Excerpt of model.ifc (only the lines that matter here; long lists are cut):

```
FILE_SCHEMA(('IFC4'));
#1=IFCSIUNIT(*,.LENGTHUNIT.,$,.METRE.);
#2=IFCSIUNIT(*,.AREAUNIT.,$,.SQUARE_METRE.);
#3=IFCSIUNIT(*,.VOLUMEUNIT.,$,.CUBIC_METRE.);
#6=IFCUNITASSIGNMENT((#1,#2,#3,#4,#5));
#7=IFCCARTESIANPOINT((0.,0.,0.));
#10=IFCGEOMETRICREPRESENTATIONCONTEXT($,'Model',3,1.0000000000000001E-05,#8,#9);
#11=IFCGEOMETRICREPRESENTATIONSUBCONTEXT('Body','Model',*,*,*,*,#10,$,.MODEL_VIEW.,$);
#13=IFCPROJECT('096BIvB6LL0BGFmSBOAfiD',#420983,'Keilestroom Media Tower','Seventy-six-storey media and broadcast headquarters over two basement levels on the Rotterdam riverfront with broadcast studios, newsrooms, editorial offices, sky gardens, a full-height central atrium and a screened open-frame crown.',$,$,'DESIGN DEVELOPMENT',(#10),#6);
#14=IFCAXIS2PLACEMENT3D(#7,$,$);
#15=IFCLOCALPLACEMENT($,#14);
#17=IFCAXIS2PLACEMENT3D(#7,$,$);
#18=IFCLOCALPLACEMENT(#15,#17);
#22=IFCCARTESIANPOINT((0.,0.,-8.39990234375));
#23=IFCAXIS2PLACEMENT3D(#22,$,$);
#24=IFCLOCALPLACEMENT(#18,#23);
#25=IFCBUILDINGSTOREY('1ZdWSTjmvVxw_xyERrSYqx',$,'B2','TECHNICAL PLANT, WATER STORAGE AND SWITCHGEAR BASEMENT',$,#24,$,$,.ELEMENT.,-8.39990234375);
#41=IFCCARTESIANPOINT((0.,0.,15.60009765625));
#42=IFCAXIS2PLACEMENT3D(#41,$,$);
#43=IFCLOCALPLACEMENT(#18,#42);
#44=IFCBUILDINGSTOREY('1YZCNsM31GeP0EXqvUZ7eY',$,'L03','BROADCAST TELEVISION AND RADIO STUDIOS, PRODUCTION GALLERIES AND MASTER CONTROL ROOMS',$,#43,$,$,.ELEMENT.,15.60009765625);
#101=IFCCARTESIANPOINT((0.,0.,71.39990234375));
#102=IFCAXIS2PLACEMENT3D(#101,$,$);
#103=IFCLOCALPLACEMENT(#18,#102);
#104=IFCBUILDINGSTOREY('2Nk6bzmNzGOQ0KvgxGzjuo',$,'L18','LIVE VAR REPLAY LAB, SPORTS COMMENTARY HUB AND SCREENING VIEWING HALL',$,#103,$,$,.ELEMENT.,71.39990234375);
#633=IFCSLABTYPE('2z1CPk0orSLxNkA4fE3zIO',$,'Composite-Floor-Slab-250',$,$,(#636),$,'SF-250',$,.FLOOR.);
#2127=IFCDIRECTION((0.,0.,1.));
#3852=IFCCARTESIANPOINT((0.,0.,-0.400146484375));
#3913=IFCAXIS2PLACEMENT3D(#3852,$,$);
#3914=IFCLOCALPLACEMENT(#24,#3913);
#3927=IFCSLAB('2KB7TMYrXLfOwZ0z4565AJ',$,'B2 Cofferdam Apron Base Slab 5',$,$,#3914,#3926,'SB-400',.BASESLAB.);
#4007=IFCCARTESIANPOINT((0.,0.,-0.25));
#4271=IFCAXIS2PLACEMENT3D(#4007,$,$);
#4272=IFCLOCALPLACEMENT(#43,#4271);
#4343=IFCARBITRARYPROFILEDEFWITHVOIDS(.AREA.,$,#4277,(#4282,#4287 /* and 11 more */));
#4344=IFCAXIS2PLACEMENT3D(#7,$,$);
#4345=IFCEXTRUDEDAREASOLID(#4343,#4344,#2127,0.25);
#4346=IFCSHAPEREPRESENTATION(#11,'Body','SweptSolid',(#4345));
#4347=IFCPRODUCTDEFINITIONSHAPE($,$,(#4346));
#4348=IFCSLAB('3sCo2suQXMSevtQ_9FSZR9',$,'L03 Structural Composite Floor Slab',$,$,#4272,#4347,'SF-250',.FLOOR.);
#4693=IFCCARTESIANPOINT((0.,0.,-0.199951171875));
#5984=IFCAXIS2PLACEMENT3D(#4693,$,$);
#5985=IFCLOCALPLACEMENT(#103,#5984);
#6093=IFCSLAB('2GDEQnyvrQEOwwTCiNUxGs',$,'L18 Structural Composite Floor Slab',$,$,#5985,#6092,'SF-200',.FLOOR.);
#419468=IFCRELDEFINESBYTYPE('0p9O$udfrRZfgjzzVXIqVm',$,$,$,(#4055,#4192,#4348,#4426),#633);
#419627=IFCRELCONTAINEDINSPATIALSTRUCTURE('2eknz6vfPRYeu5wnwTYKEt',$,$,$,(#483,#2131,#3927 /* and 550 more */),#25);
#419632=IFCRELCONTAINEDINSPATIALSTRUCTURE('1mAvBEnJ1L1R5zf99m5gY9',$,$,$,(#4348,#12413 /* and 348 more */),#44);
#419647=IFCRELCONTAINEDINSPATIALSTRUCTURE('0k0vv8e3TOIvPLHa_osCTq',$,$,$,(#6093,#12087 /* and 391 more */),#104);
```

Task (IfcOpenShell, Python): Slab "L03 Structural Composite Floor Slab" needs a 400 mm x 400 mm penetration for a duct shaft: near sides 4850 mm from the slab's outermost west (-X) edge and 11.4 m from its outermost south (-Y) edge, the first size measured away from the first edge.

```python
import numpy as np
import ifcopenshell
import ifcopenshell.api.feature
import ifcopenshell.api.geometry
import ifcopenshell.api.root
import ifcopenshell.geom
import ifcopenshell.util.placement
import ifcopenshell.util.representation
import ifcopenshell.util.shape
import ifcopenshell.util.unit

model = ifcopenshell.open("model.ifc")
unit_scale = ifcopenshell.util.unit.calculate_unit_scale(model)
settings = ifcopenshell.geom.settings()


def volume(element):
    """Net volume in cubic metres, openings subtracted."""
    shape = ifcopenshell.geom.create_shape(settings, element)
    return ifcopenshell.util.shape.get_volume(shape.geometry)


slab = model.by_guid("3sCo2suQXMSevtQ_9FSZR9")
before = volume(slab)

# Extent in the slab's own axes, in metres. The edges named are its -X and -Y sides.
slab_shape = ifcopenshell.geom.create_shape(settings, slab)
vertices = ifcopenshell.util.shape.get_vertices(slab_shape.geometry)
x_min, y_min, bottom = vertices.min(axis=0)
top = vertices[:, 2].max()

opening = ifcopenshell.api.root.create_entity(model, ifc_class="IfcOpeningElement", name="Duct shaft opening", predefined_type="OPENING")
context = ifcopenshell.util.representation.get_context(model, "Model", "Body", "MODEL_VIEW")
width, depth = 0.4, 0.4
outline = [(0.0, 0.0), (width, 0.0), (width, depth), (0.0, depth), (0.0, 0.0)]
# Overshoot both faces by 50 mm so the cut is clean.
shape = ifcopenshell.api.geometry.add_slab_representation(
    model, context=context, depth=top - bottom + 0.1, polyline=outline
)
ifcopenshell.api.geometry.assign_representation(model, product=opening, representation=shape)

matrix = ifcopenshell.util.placement.get_local_placement(slab.ObjectPlacement)
matrix[:, 3] = matrix @ np.append(np.array([x_min + 4.85, y_min + 11.4, bottom - 0.05]) / unit_scale, 1.0)
ifcopenshell.api.geometry.edit_object_placement(model, product=opening, matrix=matrix, is_si=False)
ifcopenshell.api.feature.add_feature(model, feature=opening, element=slab)

after = volume(slab)

print(f"slab volume {before:.3f} -> {after:.3f} m3")

model.write("model_rev.ifc")
```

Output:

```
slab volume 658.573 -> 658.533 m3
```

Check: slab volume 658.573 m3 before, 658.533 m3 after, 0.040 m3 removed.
